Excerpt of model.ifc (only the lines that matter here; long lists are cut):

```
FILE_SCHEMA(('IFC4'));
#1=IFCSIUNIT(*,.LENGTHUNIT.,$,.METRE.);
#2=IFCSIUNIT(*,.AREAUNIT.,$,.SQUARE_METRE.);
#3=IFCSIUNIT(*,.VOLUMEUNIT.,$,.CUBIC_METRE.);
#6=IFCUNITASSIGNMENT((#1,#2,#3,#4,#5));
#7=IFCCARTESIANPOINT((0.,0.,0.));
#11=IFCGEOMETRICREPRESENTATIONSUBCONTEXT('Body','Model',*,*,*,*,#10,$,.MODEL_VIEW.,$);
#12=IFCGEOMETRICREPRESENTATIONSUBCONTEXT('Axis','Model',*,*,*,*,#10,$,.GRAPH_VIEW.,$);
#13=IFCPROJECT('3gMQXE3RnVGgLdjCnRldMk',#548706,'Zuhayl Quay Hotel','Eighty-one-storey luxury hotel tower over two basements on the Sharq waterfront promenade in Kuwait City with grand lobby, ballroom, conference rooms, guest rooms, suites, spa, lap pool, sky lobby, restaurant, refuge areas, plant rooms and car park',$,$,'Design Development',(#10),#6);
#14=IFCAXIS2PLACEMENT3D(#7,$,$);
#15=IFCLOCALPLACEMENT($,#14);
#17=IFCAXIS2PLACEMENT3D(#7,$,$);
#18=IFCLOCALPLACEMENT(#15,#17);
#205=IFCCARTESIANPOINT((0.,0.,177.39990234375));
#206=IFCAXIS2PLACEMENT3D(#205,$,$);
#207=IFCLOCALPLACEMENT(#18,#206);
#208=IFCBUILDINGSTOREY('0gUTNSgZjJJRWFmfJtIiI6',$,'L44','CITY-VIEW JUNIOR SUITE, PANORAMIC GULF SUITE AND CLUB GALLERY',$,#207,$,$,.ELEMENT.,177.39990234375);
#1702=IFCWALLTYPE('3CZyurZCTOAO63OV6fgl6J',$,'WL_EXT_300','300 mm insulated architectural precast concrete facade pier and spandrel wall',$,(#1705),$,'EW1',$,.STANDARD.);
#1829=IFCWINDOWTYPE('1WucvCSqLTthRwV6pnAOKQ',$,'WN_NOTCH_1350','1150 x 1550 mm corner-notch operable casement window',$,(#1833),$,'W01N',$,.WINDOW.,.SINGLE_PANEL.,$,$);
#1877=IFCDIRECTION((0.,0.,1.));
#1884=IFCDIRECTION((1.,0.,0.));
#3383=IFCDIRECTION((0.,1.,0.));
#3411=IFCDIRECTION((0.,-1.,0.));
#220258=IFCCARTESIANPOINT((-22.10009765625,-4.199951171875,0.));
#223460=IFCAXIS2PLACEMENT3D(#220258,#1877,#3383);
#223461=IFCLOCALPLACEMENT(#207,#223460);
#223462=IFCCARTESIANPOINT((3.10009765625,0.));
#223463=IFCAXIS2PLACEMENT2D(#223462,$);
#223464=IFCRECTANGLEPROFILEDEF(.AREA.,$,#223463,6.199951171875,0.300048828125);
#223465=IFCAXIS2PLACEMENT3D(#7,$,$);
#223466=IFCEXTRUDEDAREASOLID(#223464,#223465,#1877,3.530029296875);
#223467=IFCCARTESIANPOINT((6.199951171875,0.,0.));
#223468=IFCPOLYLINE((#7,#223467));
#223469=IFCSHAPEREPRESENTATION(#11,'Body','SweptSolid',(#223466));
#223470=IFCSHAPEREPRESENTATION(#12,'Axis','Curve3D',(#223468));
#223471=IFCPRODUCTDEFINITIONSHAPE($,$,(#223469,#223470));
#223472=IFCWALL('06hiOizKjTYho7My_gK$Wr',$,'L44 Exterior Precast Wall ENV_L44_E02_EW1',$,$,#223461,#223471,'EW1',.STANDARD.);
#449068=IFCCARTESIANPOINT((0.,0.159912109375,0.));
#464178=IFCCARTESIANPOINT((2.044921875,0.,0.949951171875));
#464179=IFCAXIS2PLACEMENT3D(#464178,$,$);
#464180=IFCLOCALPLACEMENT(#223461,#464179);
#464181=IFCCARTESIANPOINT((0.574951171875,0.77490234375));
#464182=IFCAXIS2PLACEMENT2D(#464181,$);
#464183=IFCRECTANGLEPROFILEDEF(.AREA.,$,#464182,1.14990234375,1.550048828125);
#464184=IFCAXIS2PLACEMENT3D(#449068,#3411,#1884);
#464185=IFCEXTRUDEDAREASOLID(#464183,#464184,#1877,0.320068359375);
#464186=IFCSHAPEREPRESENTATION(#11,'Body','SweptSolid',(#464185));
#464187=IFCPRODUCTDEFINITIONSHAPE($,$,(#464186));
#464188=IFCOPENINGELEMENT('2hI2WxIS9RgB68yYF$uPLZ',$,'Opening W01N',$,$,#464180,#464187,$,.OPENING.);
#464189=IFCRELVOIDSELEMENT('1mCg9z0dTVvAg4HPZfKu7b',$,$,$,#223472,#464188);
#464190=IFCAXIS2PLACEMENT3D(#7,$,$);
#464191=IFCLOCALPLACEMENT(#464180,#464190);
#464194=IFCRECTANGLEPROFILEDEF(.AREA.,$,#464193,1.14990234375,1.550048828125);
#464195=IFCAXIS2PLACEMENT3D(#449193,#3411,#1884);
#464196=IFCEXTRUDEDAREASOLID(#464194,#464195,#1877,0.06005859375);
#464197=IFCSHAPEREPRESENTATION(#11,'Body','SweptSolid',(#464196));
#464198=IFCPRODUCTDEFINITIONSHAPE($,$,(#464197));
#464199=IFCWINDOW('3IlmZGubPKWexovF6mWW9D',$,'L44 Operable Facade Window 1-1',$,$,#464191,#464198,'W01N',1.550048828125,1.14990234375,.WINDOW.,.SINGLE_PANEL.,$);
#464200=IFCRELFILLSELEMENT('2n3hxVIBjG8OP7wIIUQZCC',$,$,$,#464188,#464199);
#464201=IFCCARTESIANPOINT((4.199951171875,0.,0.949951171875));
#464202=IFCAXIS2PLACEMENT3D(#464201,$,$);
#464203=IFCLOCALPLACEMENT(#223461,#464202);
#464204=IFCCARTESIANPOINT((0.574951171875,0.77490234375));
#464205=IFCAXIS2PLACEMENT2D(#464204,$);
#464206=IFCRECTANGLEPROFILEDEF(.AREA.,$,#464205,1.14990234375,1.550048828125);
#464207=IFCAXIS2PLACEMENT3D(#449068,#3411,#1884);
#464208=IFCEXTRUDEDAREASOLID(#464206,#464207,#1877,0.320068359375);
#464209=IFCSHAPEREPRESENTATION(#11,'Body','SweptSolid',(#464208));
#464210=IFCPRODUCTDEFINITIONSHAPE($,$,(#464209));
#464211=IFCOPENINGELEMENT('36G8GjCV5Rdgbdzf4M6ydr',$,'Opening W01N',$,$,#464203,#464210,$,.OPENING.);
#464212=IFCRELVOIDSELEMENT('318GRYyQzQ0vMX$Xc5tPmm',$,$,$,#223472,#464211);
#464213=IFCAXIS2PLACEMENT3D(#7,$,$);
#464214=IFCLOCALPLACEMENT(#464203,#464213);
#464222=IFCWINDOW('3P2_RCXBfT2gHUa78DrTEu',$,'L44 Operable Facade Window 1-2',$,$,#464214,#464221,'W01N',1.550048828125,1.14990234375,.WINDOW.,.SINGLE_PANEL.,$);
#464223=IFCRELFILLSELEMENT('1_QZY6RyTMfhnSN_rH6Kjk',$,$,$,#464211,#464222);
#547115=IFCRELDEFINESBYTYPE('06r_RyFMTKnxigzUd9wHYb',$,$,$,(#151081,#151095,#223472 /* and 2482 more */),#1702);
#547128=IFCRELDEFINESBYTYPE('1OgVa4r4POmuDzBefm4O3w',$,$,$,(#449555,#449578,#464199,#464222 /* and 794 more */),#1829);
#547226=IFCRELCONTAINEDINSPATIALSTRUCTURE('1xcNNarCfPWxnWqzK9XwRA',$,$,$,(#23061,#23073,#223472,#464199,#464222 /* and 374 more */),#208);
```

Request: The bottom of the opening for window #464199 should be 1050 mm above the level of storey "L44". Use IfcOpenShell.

```python
import numpy as np
import ifcopenshell
import ifcopenshell.api.geometry
import ifcopenshell.geom
import ifcopenshell.util.element
import ifcopenshell.util.placement
import ifcopenshell.util.shape
import ifcopenshell.util.unit

model = ifcopenshell.open("model.ifc")
unit_scale = ifcopenshell.util.unit.calculate_unit_scale(model)

window = model.by_id(464199)
opening = window.FillsVoids[0].RelatingOpeningElement
storey = ifcopenshell.util.element.get_container(window, ifc_class="IfcBuildingStorey")
level = ifcopenshell.util.placement.get_local_placement(storey.ObjectPlacement)[2, 3]

# The opening's origin need not be at the sill, so measure its lowest point.
shape = ifcopenshell.geom.create_shape(ifcopenshell.geom.settings(), opening)
bottom = ifcopenshell.util.shape.get_shape_bottom_elevation(shape, shape.geometry) / unit_scale
dz = level + 1.05 - bottom

shift = np.array([0.0, 0.0, dz])
# The window is placed relative to its opening, so it follows when the opening moves.
matrix = ifcopenshell.util.placement.get_local_placement(opening.ObjectPlacement)
matrix[:3, 3] += shift
ifcopenshell.api.geometry.edit_object_placement(
    model, product=opening, matrix=matrix, is_si=False, should_transform_children=True
)

print(f"moved by {dz * unit_scale:+.3f} m")

model.write("model_rev.ifc")
```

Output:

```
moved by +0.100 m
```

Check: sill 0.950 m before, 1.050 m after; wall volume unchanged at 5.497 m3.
